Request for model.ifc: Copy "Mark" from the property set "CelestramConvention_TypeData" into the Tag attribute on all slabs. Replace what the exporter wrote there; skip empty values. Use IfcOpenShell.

First a look at what the model holds.

```python
import ifcopenshell
import ifcopenshell.util.element

model = ifcopenshell.open("model.ifc")
print(model.schema)
slabs = model.by_type("IfcSlab")
print(len(slabs), "slabs")
for e in slabs[:8]:
    source = ifcopenshell.util.element.get_pset(e, "CelestramConvention_TypeData", "Mark")
    target = e.Tag
    print(e.id(), repr(source), repr(target), sep=" | ")
```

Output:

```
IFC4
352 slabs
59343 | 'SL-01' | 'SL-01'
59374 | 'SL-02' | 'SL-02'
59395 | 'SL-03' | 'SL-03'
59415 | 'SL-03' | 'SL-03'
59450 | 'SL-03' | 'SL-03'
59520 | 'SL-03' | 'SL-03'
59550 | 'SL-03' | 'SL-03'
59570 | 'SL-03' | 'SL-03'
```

```python
import ifcopenshell
import ifcopenshell.util.element

model = ifcopenshell.open("model.ifc")

count = 0
for e in model.by_type("IfcSlab"):
    value = ifcopenshell.util.element.get_pset(e, "CelestramConvention_TypeData", "Mark")
    current = e.Tag
    if not value or not value.strip() or current == value:
        continue
    e.Tag = value
    count += 1

print(count, "slabs updated")

model.write("model_rev.ifc")
```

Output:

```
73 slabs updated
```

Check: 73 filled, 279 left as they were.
